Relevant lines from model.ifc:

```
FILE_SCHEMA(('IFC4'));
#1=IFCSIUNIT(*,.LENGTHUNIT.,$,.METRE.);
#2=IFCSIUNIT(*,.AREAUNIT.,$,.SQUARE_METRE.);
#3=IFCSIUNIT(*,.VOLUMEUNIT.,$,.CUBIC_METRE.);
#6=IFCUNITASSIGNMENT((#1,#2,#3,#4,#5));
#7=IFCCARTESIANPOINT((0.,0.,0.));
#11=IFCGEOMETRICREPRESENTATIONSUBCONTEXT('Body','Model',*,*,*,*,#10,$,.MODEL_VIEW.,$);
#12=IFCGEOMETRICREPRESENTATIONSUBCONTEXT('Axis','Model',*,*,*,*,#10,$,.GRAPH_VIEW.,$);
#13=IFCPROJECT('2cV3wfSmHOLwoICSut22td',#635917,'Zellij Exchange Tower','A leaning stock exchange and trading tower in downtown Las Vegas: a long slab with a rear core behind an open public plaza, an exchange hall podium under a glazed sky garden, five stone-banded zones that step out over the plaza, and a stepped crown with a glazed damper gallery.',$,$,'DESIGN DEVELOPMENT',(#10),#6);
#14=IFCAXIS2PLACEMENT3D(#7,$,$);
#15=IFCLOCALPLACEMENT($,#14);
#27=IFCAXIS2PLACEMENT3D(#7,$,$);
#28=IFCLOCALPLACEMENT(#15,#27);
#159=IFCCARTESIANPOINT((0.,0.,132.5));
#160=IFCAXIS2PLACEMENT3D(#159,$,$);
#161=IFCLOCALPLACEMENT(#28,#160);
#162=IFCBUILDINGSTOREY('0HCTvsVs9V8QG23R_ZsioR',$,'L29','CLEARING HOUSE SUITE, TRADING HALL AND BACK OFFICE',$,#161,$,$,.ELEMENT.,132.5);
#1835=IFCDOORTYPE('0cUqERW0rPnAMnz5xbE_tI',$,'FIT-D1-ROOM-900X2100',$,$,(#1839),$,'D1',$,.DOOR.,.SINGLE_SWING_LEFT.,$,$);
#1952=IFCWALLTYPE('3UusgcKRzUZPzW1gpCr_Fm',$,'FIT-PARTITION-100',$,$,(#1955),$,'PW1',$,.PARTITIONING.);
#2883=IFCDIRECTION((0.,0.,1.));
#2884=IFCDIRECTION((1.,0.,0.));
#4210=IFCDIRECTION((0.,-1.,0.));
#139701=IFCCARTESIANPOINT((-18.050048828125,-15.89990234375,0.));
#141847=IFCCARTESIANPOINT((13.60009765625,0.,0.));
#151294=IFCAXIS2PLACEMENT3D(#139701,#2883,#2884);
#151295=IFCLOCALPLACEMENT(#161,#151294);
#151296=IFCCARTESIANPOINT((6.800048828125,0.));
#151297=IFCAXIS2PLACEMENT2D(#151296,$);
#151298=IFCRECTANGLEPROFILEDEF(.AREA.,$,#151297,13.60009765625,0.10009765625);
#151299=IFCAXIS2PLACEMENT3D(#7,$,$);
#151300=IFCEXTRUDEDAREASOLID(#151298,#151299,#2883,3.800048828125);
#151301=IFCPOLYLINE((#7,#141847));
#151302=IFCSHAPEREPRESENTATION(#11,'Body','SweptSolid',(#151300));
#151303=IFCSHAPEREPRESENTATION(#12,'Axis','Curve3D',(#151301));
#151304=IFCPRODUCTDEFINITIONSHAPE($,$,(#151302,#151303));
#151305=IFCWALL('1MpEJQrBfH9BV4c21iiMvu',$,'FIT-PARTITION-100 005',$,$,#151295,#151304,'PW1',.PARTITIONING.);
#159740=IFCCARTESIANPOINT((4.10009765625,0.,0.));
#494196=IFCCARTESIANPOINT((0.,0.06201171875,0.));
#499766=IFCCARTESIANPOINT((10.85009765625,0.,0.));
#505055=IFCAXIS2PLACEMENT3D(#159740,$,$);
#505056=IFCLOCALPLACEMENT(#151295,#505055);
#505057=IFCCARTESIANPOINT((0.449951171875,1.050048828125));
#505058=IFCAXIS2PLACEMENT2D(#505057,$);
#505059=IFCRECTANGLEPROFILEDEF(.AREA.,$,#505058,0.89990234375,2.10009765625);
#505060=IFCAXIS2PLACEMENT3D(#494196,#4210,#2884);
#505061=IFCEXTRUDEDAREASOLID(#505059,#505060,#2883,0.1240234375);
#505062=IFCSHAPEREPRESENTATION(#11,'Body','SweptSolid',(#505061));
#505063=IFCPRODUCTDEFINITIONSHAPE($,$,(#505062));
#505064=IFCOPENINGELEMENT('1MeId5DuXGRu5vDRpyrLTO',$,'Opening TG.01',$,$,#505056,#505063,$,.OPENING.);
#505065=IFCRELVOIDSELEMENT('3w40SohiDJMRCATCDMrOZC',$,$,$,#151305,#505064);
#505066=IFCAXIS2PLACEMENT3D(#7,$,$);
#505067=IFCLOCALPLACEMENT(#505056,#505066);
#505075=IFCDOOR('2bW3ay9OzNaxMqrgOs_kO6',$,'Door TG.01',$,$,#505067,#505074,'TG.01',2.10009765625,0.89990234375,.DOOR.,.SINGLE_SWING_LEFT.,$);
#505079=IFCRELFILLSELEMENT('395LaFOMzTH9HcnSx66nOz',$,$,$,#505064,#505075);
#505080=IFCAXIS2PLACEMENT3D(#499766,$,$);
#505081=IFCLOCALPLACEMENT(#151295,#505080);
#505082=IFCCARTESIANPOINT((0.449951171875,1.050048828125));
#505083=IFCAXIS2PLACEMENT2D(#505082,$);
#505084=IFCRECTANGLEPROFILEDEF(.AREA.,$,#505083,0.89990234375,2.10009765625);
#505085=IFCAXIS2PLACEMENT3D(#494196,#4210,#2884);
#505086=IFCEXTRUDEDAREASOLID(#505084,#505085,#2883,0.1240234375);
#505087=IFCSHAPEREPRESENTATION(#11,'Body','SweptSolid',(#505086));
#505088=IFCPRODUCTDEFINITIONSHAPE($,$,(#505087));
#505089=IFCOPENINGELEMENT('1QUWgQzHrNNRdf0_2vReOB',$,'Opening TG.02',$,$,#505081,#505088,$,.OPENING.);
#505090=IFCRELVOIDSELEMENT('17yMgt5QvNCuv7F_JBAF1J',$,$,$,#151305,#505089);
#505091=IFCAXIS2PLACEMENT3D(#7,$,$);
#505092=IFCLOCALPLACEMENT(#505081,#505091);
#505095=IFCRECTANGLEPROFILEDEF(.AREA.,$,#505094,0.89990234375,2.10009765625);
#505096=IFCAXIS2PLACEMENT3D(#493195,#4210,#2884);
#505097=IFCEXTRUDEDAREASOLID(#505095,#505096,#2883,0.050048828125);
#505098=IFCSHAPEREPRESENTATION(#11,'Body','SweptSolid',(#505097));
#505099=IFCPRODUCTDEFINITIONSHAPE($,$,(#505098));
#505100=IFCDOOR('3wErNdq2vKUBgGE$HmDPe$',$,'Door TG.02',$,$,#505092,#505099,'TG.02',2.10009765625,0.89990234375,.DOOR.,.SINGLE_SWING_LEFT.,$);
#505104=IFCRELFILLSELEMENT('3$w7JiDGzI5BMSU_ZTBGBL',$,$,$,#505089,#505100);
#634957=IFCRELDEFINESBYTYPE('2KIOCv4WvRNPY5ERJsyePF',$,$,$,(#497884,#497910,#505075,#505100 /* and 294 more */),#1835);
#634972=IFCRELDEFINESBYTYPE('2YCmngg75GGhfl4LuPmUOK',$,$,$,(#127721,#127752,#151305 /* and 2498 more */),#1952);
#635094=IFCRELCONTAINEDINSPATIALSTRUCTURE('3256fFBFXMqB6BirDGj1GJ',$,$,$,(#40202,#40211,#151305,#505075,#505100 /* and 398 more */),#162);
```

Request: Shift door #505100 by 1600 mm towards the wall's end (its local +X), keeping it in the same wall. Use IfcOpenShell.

```python
import ifcopenshell
import ifcopenshell.api.geometry
import ifcopenshell.util.placement
import ifcopenshell.util.unit

model = ifcopenshell.open("model.ifc")
unit_scale = ifcopenshell.util.unit.calculate_unit_scale(model)

door = model.by_guid("3wErNdq2vKUBgGE$HmDPe$")
opening = door.FillsVoids[0].RelatingOpeningElement
wall = opening.VoidsElements[0].RelatingBuildingElement

wall_matrix = ifcopenshell.util.placement.get_local_placement(wall.ObjectPlacement)
shift = wall_matrix[:3, 0] * 1.6 / unit_scale
before = ifcopenshell.util.placement.get_local_placement(door.ObjectPlacement)[:3, 3].copy()

# The door is placed relative to its opening, so it follows when the opening moves.
matrix = ifcopenshell.util.placement.get_local_placement(opening.ObjectPlacement)
matrix[:3, 3] += shift
ifcopenshell.api.geometry.edit_object_placement(
    model, product=opening, matrix=matrix, is_si=False, should_transform_children=True
)

after = ifcopenshell.util.placement.get_local_placement(door.ObjectPlacement)[:3, 3]
print("door moved by", (after - before).round(3) + 0.0)

model.write("model_v2.ifc")
```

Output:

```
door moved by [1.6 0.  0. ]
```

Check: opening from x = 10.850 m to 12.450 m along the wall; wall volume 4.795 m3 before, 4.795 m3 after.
